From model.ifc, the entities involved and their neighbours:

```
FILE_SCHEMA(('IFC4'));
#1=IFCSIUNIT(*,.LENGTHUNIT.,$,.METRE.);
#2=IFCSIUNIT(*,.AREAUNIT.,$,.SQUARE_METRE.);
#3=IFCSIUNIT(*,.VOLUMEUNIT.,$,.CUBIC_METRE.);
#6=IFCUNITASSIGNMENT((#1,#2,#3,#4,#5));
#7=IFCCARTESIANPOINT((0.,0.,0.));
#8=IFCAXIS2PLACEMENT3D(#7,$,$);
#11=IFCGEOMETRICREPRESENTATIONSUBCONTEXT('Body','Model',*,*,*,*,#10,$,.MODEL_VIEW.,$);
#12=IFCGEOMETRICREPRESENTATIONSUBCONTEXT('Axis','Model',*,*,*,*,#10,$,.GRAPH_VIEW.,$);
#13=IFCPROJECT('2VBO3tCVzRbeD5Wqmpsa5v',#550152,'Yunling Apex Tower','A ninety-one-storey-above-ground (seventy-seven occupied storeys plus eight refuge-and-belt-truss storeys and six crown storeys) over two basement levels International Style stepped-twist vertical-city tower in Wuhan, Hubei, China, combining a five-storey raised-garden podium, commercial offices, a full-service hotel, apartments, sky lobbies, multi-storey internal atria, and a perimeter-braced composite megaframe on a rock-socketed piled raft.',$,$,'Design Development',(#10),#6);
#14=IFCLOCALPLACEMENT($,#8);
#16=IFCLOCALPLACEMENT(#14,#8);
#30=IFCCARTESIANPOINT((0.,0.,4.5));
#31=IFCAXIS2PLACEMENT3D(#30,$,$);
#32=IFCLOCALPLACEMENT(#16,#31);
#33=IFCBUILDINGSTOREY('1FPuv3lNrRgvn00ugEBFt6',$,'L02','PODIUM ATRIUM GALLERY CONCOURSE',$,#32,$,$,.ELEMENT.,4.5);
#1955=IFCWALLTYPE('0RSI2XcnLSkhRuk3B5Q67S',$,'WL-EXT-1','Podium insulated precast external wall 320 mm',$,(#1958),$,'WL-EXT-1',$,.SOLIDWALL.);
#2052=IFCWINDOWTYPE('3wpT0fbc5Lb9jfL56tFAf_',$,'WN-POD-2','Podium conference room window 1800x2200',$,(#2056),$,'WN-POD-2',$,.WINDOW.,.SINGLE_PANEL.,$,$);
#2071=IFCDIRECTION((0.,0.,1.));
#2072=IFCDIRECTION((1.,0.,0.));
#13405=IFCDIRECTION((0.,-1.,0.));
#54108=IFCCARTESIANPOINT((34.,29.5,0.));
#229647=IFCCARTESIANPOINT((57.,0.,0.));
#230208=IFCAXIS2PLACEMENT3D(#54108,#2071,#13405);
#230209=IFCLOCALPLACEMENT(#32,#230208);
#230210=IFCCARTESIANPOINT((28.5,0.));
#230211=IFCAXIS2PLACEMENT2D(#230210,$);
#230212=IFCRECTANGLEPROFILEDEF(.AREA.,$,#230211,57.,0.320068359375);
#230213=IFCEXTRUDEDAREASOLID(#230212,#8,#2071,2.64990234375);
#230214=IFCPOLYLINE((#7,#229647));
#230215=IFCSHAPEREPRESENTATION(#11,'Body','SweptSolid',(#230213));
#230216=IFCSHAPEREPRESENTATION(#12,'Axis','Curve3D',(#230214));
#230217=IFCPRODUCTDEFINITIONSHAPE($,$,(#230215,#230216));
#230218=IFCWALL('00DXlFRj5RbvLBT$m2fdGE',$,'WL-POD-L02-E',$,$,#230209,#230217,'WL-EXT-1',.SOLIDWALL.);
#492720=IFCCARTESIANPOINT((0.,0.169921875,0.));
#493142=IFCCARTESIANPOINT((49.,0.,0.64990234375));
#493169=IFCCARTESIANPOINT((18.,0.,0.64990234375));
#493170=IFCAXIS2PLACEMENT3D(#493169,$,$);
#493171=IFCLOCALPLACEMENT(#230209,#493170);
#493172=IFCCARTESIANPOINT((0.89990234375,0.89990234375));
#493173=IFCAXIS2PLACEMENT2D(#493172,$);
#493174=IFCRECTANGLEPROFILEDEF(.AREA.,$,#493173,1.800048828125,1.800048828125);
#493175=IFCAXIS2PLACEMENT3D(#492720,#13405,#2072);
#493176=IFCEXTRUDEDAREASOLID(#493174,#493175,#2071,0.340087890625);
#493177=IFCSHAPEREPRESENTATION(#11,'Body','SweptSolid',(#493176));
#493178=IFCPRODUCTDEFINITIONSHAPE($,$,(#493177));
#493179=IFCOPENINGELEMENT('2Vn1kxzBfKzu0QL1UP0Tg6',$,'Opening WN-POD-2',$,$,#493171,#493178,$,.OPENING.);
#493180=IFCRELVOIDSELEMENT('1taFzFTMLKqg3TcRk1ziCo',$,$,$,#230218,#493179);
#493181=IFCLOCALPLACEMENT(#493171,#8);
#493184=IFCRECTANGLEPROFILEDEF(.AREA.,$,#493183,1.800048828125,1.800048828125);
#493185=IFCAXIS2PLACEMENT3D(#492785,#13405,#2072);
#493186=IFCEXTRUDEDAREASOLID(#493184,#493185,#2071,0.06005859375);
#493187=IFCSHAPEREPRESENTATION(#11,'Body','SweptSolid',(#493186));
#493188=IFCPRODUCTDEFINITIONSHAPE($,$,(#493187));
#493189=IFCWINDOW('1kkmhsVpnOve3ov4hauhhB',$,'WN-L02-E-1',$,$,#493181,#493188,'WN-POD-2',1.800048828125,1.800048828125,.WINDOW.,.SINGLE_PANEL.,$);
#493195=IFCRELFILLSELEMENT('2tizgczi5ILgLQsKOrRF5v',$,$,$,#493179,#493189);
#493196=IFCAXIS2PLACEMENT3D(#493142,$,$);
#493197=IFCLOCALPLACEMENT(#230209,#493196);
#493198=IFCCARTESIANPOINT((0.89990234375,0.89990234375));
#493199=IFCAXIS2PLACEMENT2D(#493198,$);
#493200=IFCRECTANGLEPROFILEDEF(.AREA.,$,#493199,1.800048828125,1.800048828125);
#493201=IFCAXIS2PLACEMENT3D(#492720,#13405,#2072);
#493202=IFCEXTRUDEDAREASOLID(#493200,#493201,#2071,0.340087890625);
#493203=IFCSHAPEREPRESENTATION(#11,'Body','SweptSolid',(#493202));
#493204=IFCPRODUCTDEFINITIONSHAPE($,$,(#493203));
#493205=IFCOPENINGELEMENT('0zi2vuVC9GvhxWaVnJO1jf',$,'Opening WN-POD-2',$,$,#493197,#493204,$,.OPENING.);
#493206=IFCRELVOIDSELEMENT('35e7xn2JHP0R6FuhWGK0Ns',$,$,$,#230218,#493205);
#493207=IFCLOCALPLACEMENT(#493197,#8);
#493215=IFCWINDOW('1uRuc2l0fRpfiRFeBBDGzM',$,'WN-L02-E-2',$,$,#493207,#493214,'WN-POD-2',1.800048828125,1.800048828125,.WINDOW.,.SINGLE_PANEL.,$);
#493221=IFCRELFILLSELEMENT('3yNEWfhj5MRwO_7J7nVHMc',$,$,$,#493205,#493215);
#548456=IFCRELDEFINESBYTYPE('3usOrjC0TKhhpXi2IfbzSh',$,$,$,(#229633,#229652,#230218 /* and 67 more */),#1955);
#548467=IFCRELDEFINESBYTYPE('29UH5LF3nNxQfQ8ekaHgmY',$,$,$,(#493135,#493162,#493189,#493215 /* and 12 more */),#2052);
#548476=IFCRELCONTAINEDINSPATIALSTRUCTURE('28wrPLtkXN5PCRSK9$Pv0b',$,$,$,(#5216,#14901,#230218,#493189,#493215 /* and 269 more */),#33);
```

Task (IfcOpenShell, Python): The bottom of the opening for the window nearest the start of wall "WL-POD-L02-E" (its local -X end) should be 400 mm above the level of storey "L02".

```python
import numpy as np
import ifcopenshell
import ifcopenshell.api.geometry
import ifcopenshell.geom
import ifcopenshell.util.element
import ifcopenshell.util.placement
import ifcopenshell.util.shape
import ifcopenshell.util.unit

model = ifcopenshell.open("model.ifc")
unit_scale = ifcopenshell.util.unit.calculate_unit_scale(model)

window = model.by_guid("1kkmhsVpnOve3ov4hauhhB")
opening = window.FillsVoids[0].RelatingOpeningElement
storey = ifcopenshell.util.element.get_container(window, ifc_class="IfcBuildingStorey")
level = ifcopenshell.util.placement.get_local_placement(storey.ObjectPlacement)[2, 3]

# The opening's origin need not be at the sill, so measure its lowest point.
shape = ifcopenshell.geom.create_shape(ifcopenshell.geom.settings(), opening)
bottom = ifcopenshell.util.shape.get_shape_bottom_elevation(shape, shape.geometry) / unit_scale
dz = level + 0.4 - bottom

shift = np.array([0.0, 0.0, dz])
# The window is placed relative to its opening, so it follows when the opening moves.
matrix = ifcopenshell.util.placement.get_local_placement(opening.ObjectPlacement)
matrix[:3, 3] += shift
ifcopenshell.api.geometry.edit_object_placement(
    model, product=opening, matrix=matrix, is_si=False, should_transform_children=True
)

print(f"moved by {dz * unit_scale:+.3f} m")

model.write("model_rev.ifc")
```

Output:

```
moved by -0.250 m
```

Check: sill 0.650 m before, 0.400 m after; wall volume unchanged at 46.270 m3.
